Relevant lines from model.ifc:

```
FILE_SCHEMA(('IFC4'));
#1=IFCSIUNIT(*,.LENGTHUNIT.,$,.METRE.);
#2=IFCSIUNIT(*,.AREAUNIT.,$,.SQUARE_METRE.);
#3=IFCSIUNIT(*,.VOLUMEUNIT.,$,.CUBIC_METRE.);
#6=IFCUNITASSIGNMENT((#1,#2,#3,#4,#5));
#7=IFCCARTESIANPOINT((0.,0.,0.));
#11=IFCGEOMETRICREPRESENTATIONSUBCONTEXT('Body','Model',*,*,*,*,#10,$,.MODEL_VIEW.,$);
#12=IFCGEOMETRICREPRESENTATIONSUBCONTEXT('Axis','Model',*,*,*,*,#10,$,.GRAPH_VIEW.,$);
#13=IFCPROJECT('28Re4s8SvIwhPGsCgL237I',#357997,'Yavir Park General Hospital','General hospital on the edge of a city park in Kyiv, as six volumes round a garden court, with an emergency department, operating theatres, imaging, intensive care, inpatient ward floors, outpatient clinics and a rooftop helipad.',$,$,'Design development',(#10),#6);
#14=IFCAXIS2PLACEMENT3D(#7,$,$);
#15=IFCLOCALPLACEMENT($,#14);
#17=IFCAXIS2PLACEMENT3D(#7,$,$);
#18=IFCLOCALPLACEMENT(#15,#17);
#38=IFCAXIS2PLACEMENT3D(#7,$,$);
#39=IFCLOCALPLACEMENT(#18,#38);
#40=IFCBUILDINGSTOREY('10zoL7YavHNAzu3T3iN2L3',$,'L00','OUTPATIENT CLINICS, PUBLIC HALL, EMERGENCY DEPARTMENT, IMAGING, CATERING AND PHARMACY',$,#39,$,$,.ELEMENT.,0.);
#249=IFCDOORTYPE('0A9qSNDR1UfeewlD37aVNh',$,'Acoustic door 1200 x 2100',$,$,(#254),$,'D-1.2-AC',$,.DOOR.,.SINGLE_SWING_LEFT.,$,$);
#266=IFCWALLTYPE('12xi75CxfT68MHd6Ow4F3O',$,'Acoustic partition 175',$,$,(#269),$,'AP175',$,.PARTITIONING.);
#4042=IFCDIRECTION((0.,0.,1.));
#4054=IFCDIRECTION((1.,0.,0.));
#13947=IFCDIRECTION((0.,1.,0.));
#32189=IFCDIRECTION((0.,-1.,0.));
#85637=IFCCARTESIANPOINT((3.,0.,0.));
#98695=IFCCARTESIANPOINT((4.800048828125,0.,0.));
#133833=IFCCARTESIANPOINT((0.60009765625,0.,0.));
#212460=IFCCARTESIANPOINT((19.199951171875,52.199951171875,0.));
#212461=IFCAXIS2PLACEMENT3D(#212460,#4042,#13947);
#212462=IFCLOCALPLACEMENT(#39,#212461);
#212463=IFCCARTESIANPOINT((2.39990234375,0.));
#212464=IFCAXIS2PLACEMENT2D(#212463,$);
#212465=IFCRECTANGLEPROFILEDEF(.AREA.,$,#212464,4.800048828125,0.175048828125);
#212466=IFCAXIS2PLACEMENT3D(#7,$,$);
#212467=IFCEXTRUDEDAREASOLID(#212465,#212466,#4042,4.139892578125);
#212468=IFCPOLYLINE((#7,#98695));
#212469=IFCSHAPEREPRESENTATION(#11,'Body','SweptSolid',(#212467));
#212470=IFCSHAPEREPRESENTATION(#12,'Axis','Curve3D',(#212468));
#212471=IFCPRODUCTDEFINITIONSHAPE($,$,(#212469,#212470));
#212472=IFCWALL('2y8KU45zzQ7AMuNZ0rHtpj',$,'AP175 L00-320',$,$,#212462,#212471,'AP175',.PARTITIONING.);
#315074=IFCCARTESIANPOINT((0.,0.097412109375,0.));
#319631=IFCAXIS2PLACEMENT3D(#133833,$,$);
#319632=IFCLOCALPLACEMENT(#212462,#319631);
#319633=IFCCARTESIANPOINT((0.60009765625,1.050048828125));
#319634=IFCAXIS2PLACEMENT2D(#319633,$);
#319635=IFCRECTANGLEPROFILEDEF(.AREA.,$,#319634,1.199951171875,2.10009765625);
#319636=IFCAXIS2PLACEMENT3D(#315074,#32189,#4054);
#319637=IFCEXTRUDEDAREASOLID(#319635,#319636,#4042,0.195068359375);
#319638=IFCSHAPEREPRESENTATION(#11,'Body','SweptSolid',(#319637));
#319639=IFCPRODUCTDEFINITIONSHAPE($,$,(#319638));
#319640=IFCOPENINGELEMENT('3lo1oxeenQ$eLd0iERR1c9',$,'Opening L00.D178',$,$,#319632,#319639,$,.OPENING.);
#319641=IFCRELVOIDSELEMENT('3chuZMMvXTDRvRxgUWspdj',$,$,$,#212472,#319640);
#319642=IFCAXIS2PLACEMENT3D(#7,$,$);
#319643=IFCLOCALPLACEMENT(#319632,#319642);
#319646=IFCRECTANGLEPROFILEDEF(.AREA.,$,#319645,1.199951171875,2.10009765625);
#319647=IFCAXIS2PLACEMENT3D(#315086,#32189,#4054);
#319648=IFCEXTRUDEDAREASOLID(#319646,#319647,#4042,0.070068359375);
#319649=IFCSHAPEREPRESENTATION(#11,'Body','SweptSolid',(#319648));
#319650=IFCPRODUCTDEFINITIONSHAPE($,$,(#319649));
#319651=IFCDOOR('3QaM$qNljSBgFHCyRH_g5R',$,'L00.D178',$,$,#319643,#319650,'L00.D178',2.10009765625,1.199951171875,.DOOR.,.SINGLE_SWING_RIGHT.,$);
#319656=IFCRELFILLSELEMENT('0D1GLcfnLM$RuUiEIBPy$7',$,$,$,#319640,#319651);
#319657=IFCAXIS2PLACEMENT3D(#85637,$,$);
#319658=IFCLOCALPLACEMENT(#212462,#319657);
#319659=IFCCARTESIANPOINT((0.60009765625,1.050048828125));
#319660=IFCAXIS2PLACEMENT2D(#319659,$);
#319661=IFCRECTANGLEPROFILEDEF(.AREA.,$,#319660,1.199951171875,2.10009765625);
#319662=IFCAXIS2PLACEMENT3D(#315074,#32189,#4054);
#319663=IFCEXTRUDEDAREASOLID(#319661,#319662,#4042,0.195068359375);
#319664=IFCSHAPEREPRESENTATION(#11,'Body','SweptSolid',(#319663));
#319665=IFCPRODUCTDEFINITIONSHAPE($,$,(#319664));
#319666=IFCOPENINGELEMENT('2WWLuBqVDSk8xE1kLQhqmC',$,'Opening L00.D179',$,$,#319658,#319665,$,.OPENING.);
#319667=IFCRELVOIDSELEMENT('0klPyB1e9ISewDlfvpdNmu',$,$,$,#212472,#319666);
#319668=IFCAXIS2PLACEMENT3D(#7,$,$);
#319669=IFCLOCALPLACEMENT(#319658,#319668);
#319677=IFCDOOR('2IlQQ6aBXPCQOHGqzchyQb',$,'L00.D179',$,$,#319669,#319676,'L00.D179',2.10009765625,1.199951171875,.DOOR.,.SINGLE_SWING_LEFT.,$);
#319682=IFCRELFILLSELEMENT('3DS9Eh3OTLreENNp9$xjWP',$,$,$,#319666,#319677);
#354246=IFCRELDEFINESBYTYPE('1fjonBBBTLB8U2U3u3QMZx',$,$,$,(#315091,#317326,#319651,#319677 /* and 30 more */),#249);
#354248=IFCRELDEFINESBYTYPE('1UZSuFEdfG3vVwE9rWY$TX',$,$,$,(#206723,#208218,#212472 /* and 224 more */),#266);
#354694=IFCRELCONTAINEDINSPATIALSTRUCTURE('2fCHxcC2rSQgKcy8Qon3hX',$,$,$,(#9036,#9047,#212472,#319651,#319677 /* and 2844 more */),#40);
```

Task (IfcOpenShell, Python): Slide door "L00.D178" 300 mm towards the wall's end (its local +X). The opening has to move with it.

```python
import ifcopenshell
import ifcopenshell.api.geometry
import ifcopenshell.util.placement
import ifcopenshell.util.unit

model = ifcopenshell.open("model.ifc")
unit_scale = ifcopenshell.util.unit.calculate_unit_scale(model)

door = model.by_guid("3QaM$qNljSBgFHCyRH_g5R")
opening = door.FillsVoids[0].RelatingOpeningElement
wall = opening.VoidsElements[0].RelatingBuildingElement

wall_matrix = ifcopenshell.util.placement.get_local_placement(wall.ObjectPlacement)
shift = wall_matrix[:3, 0] * 0.3 / unit_scale
before = ifcopenshell.util.placement.get_local_placement(door.ObjectPlacement)[:3, 3].copy()

# The door is placed relative to its opening, so it follows when the opening moves.
matrix = ifcopenshell.util.placement.get_local_placement(opening.ObjectPlacement)
matrix[:3, 3] += shift
ifcopenshell.api.geometry.edit_object_placement(
    model, product=opening, matrix=matrix, is_si=False, should_transform_children=True
)

after = ifcopenshell.util.placement.get_local_placement(door.ObjectPlacement)[:3, 3]
print("door moved by", (after - before).round(3) + 0.0)

model.write("model_updated.ifc")
```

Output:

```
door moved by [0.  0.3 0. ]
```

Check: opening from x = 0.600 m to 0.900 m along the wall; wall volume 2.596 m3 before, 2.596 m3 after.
